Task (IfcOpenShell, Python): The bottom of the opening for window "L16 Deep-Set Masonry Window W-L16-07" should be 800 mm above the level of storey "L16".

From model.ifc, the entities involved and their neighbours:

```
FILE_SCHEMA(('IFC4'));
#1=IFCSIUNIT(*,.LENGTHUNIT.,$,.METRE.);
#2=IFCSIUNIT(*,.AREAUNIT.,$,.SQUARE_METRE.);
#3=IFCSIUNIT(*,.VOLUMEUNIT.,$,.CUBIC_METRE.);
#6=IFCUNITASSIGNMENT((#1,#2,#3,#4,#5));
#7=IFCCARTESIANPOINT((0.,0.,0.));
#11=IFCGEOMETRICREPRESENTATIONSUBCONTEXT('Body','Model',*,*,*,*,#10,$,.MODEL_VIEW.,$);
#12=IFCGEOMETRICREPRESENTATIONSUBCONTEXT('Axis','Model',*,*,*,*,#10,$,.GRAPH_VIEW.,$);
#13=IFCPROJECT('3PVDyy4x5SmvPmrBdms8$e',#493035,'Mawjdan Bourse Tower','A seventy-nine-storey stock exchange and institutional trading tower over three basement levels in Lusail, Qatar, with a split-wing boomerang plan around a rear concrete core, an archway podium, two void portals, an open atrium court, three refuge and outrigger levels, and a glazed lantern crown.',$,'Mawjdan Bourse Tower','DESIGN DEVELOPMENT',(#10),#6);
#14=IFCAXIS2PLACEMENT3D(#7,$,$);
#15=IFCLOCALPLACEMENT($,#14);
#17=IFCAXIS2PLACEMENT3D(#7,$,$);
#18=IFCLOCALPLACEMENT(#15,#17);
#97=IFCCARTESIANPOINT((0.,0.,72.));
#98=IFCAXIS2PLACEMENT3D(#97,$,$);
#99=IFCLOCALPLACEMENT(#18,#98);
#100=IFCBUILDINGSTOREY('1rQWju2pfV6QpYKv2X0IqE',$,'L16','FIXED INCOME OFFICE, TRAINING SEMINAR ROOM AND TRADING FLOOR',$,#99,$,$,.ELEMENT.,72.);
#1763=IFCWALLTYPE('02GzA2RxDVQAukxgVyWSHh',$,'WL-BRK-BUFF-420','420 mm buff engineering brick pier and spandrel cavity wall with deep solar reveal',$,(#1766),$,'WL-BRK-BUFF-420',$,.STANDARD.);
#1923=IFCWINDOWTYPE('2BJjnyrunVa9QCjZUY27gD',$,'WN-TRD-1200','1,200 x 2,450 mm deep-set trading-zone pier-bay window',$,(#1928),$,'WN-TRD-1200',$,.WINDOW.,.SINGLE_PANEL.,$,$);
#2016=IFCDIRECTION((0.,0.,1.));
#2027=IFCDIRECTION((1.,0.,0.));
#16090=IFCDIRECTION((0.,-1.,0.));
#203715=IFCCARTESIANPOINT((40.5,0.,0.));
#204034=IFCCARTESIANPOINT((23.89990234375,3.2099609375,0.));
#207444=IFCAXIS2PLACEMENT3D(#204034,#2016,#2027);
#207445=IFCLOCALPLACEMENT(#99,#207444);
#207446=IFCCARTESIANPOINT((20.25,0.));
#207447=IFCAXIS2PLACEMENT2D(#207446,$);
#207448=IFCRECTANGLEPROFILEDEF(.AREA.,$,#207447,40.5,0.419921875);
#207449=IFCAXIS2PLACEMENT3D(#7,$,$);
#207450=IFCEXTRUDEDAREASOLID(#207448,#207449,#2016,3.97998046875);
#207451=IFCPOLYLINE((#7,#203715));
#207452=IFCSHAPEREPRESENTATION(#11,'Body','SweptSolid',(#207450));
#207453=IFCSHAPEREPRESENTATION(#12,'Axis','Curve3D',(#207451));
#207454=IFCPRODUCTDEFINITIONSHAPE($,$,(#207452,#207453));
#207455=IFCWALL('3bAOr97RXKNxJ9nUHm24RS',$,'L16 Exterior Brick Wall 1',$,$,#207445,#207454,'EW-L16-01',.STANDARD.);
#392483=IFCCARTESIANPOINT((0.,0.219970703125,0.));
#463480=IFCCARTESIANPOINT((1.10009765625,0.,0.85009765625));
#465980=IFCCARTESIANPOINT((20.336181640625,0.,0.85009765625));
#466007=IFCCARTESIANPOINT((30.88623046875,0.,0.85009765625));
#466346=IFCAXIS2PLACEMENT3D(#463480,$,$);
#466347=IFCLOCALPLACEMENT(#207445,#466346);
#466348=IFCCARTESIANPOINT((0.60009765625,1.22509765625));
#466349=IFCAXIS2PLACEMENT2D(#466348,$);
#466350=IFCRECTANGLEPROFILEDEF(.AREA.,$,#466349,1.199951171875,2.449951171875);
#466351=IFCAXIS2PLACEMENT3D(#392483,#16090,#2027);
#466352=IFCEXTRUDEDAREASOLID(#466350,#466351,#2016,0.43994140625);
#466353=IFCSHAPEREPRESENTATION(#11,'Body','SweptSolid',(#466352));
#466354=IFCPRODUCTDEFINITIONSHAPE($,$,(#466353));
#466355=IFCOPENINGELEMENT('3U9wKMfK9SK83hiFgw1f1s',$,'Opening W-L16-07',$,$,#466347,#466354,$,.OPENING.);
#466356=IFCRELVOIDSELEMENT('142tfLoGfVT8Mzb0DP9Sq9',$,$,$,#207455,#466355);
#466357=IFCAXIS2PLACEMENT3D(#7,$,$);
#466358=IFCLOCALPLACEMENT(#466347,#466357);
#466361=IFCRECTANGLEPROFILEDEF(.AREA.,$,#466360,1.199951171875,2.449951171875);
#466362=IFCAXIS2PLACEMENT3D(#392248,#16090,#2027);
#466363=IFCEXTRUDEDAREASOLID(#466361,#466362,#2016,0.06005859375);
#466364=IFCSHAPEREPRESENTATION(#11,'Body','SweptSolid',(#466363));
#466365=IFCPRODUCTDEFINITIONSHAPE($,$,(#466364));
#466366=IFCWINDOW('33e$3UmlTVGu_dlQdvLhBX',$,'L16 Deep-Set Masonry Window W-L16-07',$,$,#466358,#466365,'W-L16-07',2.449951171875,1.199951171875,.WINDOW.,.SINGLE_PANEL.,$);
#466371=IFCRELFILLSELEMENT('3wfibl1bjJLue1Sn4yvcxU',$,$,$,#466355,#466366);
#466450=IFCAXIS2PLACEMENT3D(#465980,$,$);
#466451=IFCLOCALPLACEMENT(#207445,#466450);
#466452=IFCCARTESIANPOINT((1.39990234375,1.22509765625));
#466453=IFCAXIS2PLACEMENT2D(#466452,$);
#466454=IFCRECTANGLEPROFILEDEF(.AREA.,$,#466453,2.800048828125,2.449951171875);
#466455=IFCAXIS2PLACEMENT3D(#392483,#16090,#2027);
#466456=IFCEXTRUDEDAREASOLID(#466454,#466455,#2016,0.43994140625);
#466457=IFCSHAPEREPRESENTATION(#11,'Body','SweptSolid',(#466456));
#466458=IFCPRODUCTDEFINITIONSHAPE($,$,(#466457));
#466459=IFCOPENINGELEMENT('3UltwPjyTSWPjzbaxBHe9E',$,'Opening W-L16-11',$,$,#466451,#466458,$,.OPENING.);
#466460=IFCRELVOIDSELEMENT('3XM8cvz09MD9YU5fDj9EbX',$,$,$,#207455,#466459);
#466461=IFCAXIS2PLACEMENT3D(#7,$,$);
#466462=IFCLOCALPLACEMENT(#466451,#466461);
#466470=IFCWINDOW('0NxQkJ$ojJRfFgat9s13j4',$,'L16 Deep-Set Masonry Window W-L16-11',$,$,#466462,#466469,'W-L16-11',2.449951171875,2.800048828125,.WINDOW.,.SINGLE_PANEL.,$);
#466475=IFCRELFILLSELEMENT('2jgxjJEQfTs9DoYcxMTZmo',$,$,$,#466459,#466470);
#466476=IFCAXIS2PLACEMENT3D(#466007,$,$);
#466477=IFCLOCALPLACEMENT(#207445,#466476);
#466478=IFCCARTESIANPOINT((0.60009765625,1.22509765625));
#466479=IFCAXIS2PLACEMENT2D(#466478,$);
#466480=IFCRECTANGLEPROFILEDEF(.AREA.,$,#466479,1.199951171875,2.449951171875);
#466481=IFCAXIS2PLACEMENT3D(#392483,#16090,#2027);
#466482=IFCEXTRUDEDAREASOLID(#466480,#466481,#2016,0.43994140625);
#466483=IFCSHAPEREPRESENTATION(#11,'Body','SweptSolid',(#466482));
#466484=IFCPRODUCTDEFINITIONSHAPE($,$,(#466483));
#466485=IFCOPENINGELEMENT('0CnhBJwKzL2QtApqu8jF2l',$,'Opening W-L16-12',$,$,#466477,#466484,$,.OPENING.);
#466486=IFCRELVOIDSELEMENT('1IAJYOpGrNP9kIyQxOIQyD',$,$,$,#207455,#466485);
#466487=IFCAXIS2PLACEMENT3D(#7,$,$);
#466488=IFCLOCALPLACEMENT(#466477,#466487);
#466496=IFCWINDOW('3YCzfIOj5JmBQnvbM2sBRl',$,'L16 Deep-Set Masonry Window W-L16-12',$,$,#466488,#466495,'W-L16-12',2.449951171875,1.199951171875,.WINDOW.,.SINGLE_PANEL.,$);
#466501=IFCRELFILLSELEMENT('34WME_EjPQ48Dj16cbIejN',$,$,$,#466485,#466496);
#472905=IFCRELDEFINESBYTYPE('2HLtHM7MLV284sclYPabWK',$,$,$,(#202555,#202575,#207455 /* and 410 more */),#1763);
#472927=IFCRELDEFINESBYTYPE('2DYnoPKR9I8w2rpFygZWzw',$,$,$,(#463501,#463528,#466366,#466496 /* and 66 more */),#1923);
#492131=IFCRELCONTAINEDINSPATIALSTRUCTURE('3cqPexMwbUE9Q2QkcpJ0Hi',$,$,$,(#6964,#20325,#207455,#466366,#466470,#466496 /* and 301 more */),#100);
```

```python
import numpy as np
import ifcopenshell
import ifcopenshell.api.geometry
import ifcopenshell.geom
import ifcopenshell.util.element
import ifcopenshell.util.placement
import ifcopenshell.util.shape
import ifcopenshell.util.unit

model = ifcopenshell.open("model.ifc")
unit_scale = ifcopenshell.util.unit.calculate_unit_scale(model)

window = model.by_guid("33e$3UmlTVGu_dlQdvLhBX")
opening = window.FillsVoids[0].RelatingOpeningElement
storey = ifcopenshell.util.element.get_container(window, ifc_class="IfcBuildingStorey")
level = ifcopenshell.util.placement.get_local_placement(storey.ObjectPlacement)[2, 3]

# The opening's origin need not be at the sill, so measure its lowest point.
shape = ifcopenshell.geom.create_shape(ifcopenshell.geom.settings(), opening)
bottom = ifcopenshell.util.shape.get_shape_bottom_elevation(shape, shape.geometry) / unit_scale
dz = level + 0.8 / unit_scale - bottom

shift = np.array([0.0, 0.0, dz])
# The window is placed relative to its opening, so it follows when the opening moves.
matrix = ifcopenshell.util.placement.get_local_placement(opening.ObjectPlacement)
matrix[:3, 3] += shift
ifcopenshell.api.geometry.edit_object_placement(
    model, product=opening, matrix=matrix, is_si=False, should_transform_children=True
)

print(f"moved by {dz * unit_scale:+.3f} m")

model.write("model-out.ifc")
```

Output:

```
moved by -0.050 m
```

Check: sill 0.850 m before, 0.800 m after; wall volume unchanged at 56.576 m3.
